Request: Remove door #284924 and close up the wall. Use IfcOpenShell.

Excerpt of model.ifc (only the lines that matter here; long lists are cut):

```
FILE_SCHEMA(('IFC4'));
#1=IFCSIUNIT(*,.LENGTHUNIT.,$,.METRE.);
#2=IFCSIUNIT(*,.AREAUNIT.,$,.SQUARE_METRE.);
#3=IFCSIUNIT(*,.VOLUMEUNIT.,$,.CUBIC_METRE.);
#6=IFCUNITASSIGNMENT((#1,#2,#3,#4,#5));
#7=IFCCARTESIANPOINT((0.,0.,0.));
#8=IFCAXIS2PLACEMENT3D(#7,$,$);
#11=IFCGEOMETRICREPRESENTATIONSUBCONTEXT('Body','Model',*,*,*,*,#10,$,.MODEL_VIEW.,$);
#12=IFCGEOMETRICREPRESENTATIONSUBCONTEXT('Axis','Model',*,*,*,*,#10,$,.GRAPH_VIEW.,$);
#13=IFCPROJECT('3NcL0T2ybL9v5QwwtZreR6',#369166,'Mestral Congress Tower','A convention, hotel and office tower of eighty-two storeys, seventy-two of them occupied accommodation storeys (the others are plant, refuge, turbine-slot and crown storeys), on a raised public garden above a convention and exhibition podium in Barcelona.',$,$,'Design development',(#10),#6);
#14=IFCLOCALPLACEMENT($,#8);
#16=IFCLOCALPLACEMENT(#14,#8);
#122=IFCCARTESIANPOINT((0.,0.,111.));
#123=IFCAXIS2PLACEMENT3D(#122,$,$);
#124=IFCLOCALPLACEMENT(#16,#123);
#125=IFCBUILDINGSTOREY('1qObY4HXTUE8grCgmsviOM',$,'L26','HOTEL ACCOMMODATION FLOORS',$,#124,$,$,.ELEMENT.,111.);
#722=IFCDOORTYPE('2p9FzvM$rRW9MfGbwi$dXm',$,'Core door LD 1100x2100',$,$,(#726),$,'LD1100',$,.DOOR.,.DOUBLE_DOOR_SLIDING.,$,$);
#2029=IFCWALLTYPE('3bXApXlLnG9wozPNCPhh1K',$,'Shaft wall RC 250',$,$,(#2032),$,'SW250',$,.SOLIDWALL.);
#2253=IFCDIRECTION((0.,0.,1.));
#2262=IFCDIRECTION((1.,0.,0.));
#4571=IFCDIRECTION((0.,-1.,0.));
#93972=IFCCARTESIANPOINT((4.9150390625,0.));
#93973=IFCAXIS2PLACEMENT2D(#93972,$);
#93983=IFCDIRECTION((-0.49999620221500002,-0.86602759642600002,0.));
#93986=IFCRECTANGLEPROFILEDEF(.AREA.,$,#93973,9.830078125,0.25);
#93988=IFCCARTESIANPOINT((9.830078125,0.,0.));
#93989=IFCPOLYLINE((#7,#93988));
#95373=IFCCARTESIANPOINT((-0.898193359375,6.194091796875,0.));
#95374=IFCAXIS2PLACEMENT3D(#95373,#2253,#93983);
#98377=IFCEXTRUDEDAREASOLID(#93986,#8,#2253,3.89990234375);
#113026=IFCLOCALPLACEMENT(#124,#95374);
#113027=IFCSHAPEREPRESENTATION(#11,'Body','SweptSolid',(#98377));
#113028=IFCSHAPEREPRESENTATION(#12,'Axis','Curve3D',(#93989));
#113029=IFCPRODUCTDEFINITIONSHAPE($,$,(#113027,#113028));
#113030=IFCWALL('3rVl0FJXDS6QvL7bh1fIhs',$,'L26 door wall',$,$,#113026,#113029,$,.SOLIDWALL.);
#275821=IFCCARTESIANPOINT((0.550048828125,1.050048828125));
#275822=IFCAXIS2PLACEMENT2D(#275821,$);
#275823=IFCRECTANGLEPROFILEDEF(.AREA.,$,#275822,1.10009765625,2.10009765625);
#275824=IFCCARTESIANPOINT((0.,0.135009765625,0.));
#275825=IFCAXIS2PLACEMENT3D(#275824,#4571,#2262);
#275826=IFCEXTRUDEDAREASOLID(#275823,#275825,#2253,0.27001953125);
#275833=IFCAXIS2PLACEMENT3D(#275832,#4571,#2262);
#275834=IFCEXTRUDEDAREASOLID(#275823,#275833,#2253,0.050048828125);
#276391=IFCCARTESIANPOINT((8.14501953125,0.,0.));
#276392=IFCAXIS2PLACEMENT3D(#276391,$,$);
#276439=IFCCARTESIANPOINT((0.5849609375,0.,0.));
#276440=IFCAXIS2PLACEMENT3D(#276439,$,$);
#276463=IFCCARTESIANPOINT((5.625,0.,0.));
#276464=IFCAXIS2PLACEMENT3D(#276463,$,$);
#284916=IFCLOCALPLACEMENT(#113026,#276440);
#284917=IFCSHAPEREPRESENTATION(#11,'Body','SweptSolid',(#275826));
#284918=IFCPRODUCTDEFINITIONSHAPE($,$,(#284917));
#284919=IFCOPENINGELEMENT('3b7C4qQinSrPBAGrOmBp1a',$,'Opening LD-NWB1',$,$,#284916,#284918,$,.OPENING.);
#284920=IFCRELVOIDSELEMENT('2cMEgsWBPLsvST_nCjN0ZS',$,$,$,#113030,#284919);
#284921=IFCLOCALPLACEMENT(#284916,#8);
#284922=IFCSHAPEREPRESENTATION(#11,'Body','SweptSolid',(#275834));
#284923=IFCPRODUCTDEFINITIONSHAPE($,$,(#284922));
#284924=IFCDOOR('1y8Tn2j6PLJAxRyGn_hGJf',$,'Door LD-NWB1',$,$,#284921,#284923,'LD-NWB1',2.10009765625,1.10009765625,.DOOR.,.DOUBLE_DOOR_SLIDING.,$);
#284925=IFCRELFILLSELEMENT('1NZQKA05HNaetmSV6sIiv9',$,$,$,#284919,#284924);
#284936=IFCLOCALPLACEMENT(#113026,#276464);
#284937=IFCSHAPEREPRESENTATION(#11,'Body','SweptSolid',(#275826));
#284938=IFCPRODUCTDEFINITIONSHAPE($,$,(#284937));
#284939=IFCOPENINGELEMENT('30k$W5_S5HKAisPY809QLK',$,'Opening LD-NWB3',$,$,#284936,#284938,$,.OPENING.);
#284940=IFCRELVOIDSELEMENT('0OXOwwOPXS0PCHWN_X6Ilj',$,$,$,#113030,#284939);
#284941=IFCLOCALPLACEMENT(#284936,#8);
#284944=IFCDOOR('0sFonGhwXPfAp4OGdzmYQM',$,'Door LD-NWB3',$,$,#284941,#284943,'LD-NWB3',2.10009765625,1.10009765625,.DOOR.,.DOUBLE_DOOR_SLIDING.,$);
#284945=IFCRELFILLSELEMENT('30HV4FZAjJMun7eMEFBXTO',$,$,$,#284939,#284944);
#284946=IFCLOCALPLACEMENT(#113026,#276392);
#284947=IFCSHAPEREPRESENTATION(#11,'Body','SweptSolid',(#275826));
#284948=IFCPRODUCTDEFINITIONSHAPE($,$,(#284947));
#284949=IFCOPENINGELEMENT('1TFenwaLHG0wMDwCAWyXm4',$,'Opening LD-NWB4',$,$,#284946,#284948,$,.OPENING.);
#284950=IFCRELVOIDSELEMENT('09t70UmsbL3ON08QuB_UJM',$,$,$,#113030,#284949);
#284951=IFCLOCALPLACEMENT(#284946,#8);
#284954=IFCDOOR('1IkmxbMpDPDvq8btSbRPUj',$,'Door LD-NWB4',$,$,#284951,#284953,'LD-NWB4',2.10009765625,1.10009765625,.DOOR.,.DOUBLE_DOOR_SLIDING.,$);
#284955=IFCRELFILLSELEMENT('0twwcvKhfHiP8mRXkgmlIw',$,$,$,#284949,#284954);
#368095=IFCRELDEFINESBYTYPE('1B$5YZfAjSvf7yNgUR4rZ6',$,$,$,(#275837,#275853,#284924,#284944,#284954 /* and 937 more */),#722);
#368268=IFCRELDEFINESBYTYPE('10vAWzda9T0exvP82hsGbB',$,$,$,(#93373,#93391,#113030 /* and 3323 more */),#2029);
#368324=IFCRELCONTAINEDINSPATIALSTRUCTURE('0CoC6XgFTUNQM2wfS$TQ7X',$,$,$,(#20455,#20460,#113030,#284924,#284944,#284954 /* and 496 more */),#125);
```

```python
import ifcopenshell
import ifcopenshell.api.feature
import ifcopenshell.api.root
import ifcopenshell.geom
import ifcopenshell.util.shape

model = ifcopenshell.open("model.ifc")
settings = ifcopenshell.geom.settings()


def volume(element):
    """Net volume in cubic metres, openings subtracted."""
    shape = ifcopenshell.geom.create_shape(settings, element)
    return ifcopenshell.util.shape.get_volume(shape.geometry)


door = model.by_id(284924)
opening = door.FillsVoids[0].RelatingOpeningElement
wall = opening.VoidsElements[0].RelatingBuildingElement
before = volume(wall)

ifcopenshell.api.root.remove_product(model, product=door)
ifcopenshell.api.feature.remove_feature(model, feature=opening)

after = volume(wall)

print(f"wall volume {before:.3f} -> {after:.3f} m3")

model.write("model-out.ifc")
```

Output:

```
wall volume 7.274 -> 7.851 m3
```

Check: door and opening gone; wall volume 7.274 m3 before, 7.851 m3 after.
